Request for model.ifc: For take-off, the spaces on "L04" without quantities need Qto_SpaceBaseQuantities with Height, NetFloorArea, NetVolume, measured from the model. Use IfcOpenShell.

First a look at what the model holds.

```python
import ifcopenshell
import ifcopenshell.util.element
import ifcopenshell.util.unit

model = ifcopenshell.open("model.ifc")
print(model.schema)
for unit_type in ("LENGTHUNIT", "AREAUNIT", "VOLUMEUNIT"):
    print(unit_type, ifcopenshell.util.unit.calculate_unit_scale(model, unit_type))
storey = next(s for s in model.by_type("IfcBuildingStorey") if s.Name == "L04")
spaces = [e for e in ifcopenshell.util.element.get_decomposition(storey) if e.is_a("IfcSpace")]
for e in sorted(spaces, key=lambda e: e.id()):
    print(e.id(), e.is_a(), e.Name, list(ifcopenshell.util.element.get_psets(e, qtos_only=True)), sep=" | ")
```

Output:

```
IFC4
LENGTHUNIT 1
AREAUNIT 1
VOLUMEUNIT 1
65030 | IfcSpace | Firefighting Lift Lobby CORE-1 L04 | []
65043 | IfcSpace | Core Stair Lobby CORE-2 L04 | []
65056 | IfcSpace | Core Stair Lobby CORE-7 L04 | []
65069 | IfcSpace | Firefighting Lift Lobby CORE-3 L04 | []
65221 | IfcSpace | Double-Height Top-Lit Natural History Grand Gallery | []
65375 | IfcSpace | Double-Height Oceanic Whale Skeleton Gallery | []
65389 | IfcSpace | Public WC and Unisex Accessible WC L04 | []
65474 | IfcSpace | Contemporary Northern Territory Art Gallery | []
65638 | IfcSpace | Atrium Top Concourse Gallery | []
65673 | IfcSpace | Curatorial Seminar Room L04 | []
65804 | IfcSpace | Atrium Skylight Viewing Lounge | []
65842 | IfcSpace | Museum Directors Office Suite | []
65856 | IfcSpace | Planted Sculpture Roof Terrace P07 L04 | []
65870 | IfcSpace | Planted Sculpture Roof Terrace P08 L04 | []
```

```python
import ifcopenshell
import ifcopenshell.api.pset
import ifcopenshell.geom
import ifcopenshell.util.element
import ifcopenshell.util.shape
import ifcopenshell.util.unit

model = ifcopenshell.open("model.ifc")
unit_scale = ifcopenshell.util.unit.calculate_unit_scale(model)
area_scale = ifcopenshell.util.unit.calculate_unit_scale(model, "AREAUNIT")
volume_scale = ifcopenshell.util.unit.calculate_unit_scale(model, "VOLUMEUNIT")
settings = ifcopenshell.geom.settings()

storey = next(s for s in model.by_type("IfcBuildingStorey") if s.Name == "L04")
spaces = [e for e in ifcopenshell.util.element.get_decomposition(storey) if e.is_a("IfcSpace")]

for e in sorted(spaces, key=lambda e: e.id()):
    if ifcopenshell.util.element.get_psets(e, qtos_only=True, should_inherit=False):
        continue
    # Geometry comes back in metres, in the element's own axes.
    shape = ifcopenshell.geom.create_shape(settings, e)
    values = {
        "Height": ifcopenshell.util.shape.get_z(shape.geometry) / unit_scale,
        "NetFloorArea": ifcopenshell.util.shape.get_footprint_area(shape.geometry) / area_scale,
        "NetVolume": ifcopenshell.util.shape.get_volume(shape.geometry) / volume_scale,
    }
    qto = ifcopenshell.api.pset.add_qto(model, product=e, name="Qto_SpaceBaseQuantities")
    ifcopenshell.api.pset.edit_qto(model, qto=qto, properties=values)
    print(e.id(), {k: round(v, 3) for k, v in values.items()})

model.write("model_updated.ifc")
```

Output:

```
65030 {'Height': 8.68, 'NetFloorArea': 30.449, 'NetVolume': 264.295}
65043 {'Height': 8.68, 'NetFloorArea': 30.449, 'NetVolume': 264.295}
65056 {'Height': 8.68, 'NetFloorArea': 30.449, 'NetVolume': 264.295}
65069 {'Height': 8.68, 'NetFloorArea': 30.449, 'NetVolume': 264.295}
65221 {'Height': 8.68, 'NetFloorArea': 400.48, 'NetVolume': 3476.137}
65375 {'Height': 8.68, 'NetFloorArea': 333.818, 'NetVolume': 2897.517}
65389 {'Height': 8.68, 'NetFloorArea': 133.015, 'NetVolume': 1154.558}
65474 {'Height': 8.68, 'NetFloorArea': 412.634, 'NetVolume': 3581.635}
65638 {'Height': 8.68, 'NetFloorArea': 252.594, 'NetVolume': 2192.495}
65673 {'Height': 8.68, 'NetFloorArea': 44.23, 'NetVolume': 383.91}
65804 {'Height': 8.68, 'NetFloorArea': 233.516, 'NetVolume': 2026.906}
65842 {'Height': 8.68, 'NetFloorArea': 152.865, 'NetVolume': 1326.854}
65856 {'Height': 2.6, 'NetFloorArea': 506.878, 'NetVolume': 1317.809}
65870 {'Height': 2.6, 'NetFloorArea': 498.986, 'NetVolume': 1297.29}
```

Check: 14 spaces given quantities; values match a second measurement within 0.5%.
